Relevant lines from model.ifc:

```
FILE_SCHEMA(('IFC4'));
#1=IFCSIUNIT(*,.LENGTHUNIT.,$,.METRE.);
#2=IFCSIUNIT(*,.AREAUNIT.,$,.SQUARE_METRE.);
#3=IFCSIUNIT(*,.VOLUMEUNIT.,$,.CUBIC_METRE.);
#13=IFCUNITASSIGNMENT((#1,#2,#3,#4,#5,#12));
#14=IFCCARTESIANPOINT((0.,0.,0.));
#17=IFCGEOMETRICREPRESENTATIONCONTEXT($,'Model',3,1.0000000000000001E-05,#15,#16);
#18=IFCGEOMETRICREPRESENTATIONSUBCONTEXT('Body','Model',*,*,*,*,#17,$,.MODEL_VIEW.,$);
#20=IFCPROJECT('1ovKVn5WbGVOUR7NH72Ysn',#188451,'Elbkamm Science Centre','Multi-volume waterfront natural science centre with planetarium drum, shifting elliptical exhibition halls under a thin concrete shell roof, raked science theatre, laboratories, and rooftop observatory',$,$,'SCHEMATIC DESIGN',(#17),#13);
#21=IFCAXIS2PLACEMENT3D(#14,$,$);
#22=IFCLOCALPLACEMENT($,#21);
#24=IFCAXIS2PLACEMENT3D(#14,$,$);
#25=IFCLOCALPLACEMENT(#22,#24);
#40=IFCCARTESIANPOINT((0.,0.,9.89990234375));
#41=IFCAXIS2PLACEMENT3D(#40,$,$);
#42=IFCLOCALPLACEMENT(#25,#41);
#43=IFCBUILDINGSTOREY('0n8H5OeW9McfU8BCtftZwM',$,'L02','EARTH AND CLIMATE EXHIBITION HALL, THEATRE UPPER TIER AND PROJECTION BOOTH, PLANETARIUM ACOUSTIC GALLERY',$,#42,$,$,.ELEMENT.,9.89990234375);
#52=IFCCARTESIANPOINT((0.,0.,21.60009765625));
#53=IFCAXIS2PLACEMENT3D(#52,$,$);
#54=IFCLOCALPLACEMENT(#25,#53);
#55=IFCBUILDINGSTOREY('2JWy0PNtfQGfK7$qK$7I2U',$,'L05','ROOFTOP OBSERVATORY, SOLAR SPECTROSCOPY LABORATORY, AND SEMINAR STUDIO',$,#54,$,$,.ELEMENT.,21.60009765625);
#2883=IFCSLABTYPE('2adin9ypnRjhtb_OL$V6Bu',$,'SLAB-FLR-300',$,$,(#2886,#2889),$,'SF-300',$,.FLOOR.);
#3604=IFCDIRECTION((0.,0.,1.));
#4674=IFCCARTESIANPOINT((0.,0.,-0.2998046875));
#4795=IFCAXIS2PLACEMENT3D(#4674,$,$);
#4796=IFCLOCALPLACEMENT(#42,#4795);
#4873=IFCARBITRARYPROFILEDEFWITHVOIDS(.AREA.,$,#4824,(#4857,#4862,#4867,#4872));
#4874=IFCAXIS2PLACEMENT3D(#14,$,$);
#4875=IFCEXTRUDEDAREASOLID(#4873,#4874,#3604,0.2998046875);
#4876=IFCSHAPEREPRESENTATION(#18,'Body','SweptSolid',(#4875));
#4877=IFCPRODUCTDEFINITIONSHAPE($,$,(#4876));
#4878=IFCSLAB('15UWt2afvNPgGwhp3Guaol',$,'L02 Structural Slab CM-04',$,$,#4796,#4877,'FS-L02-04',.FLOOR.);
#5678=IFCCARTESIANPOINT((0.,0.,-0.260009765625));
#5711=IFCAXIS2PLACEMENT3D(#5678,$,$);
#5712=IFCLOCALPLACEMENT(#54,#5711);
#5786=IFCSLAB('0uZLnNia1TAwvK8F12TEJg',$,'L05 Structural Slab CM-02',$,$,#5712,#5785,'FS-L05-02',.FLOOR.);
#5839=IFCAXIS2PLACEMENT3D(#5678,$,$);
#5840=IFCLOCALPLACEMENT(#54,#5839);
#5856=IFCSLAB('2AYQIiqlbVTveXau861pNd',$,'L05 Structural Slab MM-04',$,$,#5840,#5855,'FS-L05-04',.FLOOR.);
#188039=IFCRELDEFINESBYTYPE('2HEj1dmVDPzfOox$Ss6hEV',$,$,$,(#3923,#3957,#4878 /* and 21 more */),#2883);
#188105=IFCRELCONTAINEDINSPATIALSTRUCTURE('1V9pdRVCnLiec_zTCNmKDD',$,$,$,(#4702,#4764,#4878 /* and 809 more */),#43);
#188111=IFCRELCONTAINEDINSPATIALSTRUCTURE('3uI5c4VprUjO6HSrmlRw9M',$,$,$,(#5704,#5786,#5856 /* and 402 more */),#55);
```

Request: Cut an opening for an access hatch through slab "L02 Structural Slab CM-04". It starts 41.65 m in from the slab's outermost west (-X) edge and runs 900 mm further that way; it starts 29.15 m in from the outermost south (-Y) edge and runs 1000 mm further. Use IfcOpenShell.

```python
import numpy as np
import ifcopenshell
import ifcopenshell.api.feature
import ifcopenshell.api.geometry
import ifcopenshell.api.root
import ifcopenshell.geom
import ifcopenshell.util.placement
import ifcopenshell.util.representation
import ifcopenshell.util.shape
import ifcopenshell.util.unit

model = ifcopenshell.open("model.ifc")
unit_scale = ifcopenshell.util.unit.calculate_unit_scale(model)
settings = ifcopenshell.geom.settings()


def volume(element):
    """Net volume in cubic metres, openings subtracted."""
    shape = ifcopenshell.geom.create_shape(settings, element)
    return ifcopenshell.util.shape.get_volume(shape.geometry)


slab = model.by_guid("15UWt2afvNPgGwhp3Guaol")
before = volume(slab)

# Extent in the slab's own axes, in metres. The edges named are its -X and -Y sides.
slab_shape = ifcopenshell.geom.create_shape(settings, slab)
vertices = ifcopenshell.util.shape.get_vertices(slab_shape.geometry)
x_min, y_min, bottom = vertices.min(axis=0)
top = vertices[:, 2].max()

opening = ifcopenshell.api.root.create_entity(model, ifc_class="IfcOpeningElement", name="Access hatch opening", predefined_type="OPENING")
context = ifcopenshell.util.representation.get_context(model, "Model", "Body", "MODEL_VIEW")
width, depth = 0.9, 1
outline = [(0.0, 0.0), (width, 0.0), (width, depth), (0.0, depth), (0.0, 0.0)]
# Overshoot both faces by 50 mm so the cut is clean.
shape = ifcopenshell.api.geometry.add_slab_representation(
    model, context=context, depth=top - bottom + 0.1, polyline=outline
)
ifcopenshell.api.geometry.assign_representation(model, product=opening, representation=shape)

matrix = ifcopenshell.util.placement.get_local_placement(slab.ObjectPlacement)
matrix[:, 3] = matrix @ np.append(np.array([x_min + 41.65, y_min + 29.15, bottom - 0.05]) / unit_scale, 1.0)
ifcopenshell.api.geometry.edit_object_placement(model, product=opening, matrix=matrix, is_si=False)
ifcopenshell.api.feature.add_feature(model, feature=opening, element=slab)

after = volume(slab)

print(f"slab volume {before:.3f} -> {after:.3f} m3")

model.write("model_v2.ifc")
```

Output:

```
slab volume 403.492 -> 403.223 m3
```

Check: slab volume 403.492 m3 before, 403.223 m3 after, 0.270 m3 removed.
